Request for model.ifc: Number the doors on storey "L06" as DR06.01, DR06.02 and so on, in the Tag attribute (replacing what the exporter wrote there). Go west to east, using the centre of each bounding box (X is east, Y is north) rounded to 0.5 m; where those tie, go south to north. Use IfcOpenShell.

First a look at what the model holds.

```python
import ifcopenshell
import ifcopenshell.util.element
import ifcopenshell.util.placement

model = ifcopenshell.open("model.ifc")
print(model.schema)
storey = next(s for s in model.by_type("IfcBuildingStorey") if s.Name == "L06")
doors = [e for e in ifcopenshell.util.element.get_decomposition(storey) if e.is_a("IfcDoor")]
for e in sorted(doors, key=lambda e: e.id()):
    origin = ifcopenshell.util.placement.get_local_placement(e.ObjectPlacement)[:3, 3]
    print(e.id(), e.Tag, e.Name, origin.round(2) + 0.0, sep=" | ")
```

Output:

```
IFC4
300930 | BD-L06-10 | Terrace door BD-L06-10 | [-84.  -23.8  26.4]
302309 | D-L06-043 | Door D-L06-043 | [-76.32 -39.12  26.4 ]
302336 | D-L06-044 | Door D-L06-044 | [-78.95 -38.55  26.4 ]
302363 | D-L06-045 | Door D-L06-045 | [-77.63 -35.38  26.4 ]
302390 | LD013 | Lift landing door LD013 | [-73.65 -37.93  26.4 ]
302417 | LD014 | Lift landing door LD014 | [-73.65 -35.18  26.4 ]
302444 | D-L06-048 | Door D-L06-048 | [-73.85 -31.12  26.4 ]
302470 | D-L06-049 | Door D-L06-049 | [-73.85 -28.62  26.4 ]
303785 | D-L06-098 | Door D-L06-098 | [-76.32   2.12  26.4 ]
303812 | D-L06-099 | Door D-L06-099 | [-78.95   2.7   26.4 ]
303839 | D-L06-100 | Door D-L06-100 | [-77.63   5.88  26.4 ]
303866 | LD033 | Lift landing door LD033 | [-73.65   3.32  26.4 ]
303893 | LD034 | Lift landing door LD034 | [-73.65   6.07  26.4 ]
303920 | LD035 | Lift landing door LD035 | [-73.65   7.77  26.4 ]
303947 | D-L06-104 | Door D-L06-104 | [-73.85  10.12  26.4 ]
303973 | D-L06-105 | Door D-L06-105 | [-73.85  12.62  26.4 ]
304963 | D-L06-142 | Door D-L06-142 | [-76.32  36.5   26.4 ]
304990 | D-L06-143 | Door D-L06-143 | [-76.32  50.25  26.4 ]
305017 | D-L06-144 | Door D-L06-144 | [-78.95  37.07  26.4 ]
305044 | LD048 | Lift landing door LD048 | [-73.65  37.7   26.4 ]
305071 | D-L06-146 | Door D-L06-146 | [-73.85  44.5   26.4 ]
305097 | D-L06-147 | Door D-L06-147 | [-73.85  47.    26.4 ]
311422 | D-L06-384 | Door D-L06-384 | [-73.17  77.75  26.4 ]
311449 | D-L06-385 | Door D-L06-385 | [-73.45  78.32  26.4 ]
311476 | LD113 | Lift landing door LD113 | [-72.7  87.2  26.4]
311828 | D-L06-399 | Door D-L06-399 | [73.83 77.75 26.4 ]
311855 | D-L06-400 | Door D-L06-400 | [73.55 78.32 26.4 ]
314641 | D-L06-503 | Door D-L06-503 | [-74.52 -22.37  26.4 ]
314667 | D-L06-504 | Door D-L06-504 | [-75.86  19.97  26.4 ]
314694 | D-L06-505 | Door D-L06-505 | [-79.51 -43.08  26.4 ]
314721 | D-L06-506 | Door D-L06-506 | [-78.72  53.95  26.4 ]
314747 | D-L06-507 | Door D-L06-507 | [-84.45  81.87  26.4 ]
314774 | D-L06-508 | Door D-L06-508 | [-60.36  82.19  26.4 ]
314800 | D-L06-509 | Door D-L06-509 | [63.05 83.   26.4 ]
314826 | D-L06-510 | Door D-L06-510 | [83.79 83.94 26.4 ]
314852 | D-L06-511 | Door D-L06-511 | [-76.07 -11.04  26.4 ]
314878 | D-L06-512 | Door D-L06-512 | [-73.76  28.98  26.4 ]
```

```python
import ifcopenshell
import ifcopenshell.geom
import ifcopenshell.util.element
import ifcopenshell.util.shape

model = ifcopenshell.open("model.ifc")
settings = ifcopenshell.geom.settings()
settings.set("use-world-coords", True)


def centre(element):
    shape = ifcopenshell.geom.create_shape(settings, element)
    return ifcopenshell.util.shape.get_bbox_centroid(shape.geometry)


storey = next(s for s in model.by_type("IfcBuildingStorey") if s.Name == "L06")
doors = [e for e in ifcopenshell.util.element.get_decomposition(storey) if e.is_a("IfcDoor")]

# Insertion points can sit at a corner or the storey origin, so sort by the geometry (in metres).
centres = {e: centre(e) for e in doors}
doors.sort(key=lambda e: (round(centres[e][0] / 0.5), centres[e][1]))

for i, e in enumerate(doors, start=1):
    number = f"DR06.{i:02d}"
    e.Tag = number
    print(e.id(), number)

model.write("model_v2.ifc")
```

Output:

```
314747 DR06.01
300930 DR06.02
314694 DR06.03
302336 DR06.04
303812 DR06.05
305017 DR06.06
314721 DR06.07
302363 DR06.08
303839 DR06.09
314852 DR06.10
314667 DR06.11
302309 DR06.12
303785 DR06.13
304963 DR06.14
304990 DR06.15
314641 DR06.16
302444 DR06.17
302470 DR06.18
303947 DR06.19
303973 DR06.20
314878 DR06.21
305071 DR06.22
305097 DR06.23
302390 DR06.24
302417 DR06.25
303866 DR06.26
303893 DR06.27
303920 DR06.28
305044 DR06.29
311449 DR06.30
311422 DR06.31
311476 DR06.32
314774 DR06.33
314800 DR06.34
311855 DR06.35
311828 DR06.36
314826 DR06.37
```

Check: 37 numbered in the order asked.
